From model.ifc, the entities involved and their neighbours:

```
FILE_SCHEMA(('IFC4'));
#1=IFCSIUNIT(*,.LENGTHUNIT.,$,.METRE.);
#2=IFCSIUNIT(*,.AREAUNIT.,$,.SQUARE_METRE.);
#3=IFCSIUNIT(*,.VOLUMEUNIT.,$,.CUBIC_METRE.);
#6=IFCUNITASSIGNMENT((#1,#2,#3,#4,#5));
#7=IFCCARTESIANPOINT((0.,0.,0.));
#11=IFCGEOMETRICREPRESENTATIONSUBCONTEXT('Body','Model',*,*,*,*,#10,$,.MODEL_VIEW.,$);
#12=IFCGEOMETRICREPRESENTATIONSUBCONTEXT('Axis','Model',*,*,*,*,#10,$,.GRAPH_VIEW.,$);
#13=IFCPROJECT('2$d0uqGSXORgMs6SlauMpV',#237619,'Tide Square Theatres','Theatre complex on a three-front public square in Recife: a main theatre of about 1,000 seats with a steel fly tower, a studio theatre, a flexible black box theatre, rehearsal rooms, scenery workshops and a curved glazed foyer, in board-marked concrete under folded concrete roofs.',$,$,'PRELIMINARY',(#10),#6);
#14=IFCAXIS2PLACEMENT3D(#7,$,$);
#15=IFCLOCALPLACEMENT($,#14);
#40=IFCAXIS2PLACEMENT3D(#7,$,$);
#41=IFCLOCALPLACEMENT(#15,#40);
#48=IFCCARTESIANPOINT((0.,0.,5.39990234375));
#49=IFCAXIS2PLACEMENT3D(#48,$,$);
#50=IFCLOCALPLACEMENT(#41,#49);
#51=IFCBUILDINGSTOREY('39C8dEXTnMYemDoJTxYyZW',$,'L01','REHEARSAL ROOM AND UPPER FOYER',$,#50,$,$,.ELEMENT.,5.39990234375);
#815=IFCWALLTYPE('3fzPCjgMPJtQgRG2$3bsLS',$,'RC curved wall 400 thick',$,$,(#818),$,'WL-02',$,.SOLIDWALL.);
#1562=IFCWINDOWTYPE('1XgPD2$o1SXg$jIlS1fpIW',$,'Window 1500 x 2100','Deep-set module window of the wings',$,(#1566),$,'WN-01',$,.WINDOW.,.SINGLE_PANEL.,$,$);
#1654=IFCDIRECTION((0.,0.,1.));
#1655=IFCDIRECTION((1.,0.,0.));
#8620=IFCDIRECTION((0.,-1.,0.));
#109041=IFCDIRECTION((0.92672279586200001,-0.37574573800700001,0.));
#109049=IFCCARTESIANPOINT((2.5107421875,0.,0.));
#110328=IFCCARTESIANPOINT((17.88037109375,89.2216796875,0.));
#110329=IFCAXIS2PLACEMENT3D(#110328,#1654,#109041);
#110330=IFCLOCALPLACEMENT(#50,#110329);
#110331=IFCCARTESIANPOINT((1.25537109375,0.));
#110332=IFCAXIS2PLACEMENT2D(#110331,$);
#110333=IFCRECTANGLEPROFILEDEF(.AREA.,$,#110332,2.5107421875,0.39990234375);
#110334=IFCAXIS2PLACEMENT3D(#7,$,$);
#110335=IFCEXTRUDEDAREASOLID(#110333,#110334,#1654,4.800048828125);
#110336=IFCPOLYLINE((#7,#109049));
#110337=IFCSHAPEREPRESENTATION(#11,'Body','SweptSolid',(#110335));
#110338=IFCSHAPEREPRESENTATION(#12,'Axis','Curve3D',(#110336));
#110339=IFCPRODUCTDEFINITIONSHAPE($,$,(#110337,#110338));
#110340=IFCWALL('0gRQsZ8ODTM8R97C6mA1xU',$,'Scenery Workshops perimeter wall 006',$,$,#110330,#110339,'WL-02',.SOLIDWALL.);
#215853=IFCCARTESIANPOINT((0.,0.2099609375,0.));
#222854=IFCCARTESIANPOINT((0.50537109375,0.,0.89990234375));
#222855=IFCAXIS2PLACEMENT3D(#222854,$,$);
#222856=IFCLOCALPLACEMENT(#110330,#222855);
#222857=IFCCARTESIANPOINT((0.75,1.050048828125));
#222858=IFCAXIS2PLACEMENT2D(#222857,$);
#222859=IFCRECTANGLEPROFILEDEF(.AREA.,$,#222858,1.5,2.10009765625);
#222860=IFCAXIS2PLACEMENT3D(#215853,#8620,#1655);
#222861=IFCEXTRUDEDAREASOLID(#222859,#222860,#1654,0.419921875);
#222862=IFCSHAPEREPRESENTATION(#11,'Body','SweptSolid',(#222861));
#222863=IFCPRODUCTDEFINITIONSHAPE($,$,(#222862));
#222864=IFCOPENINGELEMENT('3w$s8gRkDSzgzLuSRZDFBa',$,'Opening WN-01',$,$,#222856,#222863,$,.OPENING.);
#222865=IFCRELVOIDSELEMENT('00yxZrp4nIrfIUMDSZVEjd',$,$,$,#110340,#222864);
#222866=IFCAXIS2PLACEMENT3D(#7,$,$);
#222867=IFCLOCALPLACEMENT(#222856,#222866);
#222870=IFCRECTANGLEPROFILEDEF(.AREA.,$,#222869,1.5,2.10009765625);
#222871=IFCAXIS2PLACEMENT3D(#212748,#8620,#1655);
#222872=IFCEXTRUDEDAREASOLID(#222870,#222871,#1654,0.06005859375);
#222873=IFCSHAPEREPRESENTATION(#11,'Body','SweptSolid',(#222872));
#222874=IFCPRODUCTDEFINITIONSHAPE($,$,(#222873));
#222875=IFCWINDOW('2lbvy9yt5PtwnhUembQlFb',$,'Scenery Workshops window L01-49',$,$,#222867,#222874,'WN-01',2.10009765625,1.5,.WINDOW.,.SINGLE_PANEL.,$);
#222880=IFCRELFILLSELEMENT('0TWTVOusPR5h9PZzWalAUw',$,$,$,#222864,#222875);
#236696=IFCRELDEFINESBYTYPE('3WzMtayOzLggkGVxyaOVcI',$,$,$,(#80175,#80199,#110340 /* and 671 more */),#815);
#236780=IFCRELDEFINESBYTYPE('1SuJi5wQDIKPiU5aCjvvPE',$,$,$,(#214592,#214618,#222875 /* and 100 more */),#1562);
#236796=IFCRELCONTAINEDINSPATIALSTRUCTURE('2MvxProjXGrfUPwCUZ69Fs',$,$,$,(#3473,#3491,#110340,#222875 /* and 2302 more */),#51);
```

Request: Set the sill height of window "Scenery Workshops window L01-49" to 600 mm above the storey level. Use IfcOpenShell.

```python
import numpy as np
import ifcopenshell
import ifcopenshell.api.geometry
import ifcopenshell.geom
import ifcopenshell.util.element
import ifcopenshell.util.placement
import ifcopenshell.util.shape
import ifcopenshell.util.unit

model = ifcopenshell.open("model.ifc")
unit_scale = ifcopenshell.util.unit.calculate_unit_scale(model)

window = model.by_guid("2lbvy9yt5PtwnhUembQlFb")
opening = window.FillsVoids[0].RelatingOpeningElement
storey = ifcopenshell.util.element.get_container(window, ifc_class="IfcBuildingStorey")
level = ifcopenshell.util.placement.get_local_placement(storey.ObjectPlacement)[2, 3]

# The opening's origin need not be at the sill, so measure its lowest point.
shape = ifcopenshell.geom.create_shape(ifcopenshell.geom.settings(), opening)
bottom = ifcopenshell.util.shape.get_shape_bottom_elevation(shape, shape.geometry) / unit_scale
dz = level + 0.6 - bottom

shift = np.array([0.0, 0.0, dz])
# The window is placed relative to its opening, so it follows when the opening moves.
matrix = ifcopenshell.util.placement.get_local_placement(opening.ObjectPlacement)
matrix[:3, 3] += shift
ifcopenshell.api.geometry.edit_object_placement(
    model, product=opening, matrix=matrix, is_si=False, should_transform_children=True
)

print(f"moved by {dz * unit_scale:+.3f} m")

model.write("model_rev.ifc")
```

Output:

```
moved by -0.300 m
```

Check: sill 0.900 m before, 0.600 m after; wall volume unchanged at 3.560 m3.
